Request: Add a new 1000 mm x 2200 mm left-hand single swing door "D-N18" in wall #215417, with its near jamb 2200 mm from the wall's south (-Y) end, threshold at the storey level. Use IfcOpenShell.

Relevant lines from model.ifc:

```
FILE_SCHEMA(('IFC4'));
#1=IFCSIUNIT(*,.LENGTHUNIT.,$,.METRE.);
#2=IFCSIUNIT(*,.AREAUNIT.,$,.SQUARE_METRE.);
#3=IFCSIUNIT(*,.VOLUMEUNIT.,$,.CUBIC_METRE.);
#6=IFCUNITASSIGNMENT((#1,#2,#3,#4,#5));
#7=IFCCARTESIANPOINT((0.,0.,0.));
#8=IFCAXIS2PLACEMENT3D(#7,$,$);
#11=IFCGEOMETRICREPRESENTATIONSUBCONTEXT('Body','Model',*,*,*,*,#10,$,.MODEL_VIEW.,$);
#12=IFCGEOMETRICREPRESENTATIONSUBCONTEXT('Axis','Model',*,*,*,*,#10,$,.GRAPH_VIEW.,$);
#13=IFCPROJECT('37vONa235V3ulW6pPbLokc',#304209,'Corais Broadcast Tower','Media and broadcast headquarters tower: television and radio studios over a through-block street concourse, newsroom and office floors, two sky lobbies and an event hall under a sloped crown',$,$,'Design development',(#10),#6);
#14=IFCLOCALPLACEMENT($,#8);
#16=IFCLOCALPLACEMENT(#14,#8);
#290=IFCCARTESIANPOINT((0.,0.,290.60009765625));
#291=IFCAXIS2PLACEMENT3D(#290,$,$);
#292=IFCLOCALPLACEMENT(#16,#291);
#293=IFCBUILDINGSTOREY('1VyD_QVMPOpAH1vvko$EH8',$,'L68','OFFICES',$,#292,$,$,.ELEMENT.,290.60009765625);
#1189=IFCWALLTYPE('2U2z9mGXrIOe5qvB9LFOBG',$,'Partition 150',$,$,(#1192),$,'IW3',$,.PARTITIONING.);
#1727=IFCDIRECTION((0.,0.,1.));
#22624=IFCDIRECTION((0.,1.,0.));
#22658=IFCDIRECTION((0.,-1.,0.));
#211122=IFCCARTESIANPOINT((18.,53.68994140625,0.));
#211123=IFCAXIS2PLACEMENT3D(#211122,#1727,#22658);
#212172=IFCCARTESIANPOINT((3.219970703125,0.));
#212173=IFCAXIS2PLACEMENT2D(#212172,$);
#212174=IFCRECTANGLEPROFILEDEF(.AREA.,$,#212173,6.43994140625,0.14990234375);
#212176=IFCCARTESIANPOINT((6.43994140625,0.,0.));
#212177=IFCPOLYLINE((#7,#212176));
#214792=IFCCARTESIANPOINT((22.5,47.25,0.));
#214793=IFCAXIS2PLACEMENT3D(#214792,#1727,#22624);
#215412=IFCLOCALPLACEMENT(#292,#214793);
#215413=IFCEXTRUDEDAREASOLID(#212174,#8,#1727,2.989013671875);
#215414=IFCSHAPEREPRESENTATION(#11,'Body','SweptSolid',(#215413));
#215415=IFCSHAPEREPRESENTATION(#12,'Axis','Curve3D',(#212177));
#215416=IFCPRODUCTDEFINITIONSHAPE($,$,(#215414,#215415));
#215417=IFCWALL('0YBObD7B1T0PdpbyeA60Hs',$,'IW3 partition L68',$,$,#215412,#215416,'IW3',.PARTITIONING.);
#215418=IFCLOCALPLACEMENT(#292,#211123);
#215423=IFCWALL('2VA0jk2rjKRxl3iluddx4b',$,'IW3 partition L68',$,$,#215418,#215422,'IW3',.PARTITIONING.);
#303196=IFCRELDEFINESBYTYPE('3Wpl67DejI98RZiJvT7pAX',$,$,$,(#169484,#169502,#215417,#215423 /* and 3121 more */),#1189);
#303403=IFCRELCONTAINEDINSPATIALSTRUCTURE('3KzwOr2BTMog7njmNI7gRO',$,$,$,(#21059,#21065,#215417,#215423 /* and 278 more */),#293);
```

```python
import numpy as np
import ifcopenshell
import ifcopenshell.api.feature
import ifcopenshell.api.geometry
import ifcopenshell.api.root
import ifcopenshell.api.spatial
import ifcopenshell.geom
import ifcopenshell.util.element
import ifcopenshell.util.placement
import ifcopenshell.util.representation
import ifcopenshell.util.shape
import ifcopenshell.util.unit

model = ifcopenshell.open("model.ifc")
unit_scale = ifcopenshell.util.unit.calculate_unit_scale(model)
settings = ifcopenshell.geom.settings()


def volume(element):
    """Net volume in cubic metres, openings subtracted."""
    shape = ifcopenshell.geom.create_shape(settings, element)
    return ifcopenshell.util.shape.get_volume(shape.geometry)


wall = model.by_guid("0YBObD7B1T0PdpbyeA60Hs")
storey = ifcopenshell.util.element.get_container(wall, ifc_class="IfcBuildingStorey")
context = ifcopenshell.util.representation.get_context(model, "Model", "Body", "MODEL_VIEW")
before = volume(wall)

width, height, from_end, sill = 1, 2.2, 2.2, 0.0  # metres

# The wall runs along its own X axis, and the end named is its -X end.
wall_shape = ifcopenshell.geom.create_shape(settings, wall)
x, y, z = ifcopenshell.util.shape.get_vertices(wall_shape.geometry).T
start = x.min() + from_end
face, thickness = float(y.min()), float(y.max() - y.min())
wall_matrix = ifcopenshell.util.placement.get_local_placement(wall.ObjectPlacement)
level = ifcopenshell.util.placement.get_local_placement(storey.ObjectPlacement)[2, 3]


def in_wall(x, y):
    """Placement at x, y metres in the wall's axes, at sill height."""
    matrix = wall_matrix.copy()
    matrix[:, 3] = wall_matrix @ np.array([x / unit_scale, y / unit_scale, 0.0, 1.0])
    matrix[2, 3] = level + sill / unit_scale
    return matrix


# Opening: a box that overshoots both wall faces by 50 mm.
opening = ifcopenshell.api.root.create_entity(model, ifc_class="IfcOpeningElement", predefined_type="OPENING")
box = ifcopenshell.api.geometry.add_wall_representation(
    model, context=context, length=width, height=height, thickness=thickness + 0.1
)
ifcopenshell.api.geometry.assign_representation(model, product=opening, representation=box)
ifcopenshell.api.geometry.edit_object_placement(model, product=opening, matrix=in_wall(start, face - 0.05), is_si=False)
ifcopenshell.api.feature.add_feature(model, feature=opening, element=wall)

door = ifcopenshell.api.root.create_entity(model, ifc_class="IfcDoor", name="D-N18", predefined_type="DOOR")
door.OverallWidth, door.OverallHeight = width / unit_scale, height / unit_scale
door.OperationType = "SINGLE_SWING_LEFT"
body = ifcopenshell.api.geometry.add_door_representation(
    model,
    context=context,
    overall_width=door.OverallWidth,
    overall_height=door.OverallHeight,
    operation_type="SINGLE_SWING_LEFT",
    lining_properties={"LiningDepth": thickness / unit_scale, "ThresholdDepth": thickness / unit_scale},
)
ifcopenshell.api.geometry.assign_representation(model, product=door, representation=body)
ifcopenshell.api.spatial.assign_container(model, products=[door], relating_structure=storey)
ifcopenshell.api.feature.add_filling(model, opening=opening, element=door)

# The lining spans the wall, so the door starts at the wall face.
ifcopenshell.api.geometry.edit_object_placement(model, product=door, matrix=in_wall(start, face), is_si=False)

after = volume(wall)

print(f"wall volume {before:.3f} -> {after:.3f} m3")

model.write("model_rev.ifc")
```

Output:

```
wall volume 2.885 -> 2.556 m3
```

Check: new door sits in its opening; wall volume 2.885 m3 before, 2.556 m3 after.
